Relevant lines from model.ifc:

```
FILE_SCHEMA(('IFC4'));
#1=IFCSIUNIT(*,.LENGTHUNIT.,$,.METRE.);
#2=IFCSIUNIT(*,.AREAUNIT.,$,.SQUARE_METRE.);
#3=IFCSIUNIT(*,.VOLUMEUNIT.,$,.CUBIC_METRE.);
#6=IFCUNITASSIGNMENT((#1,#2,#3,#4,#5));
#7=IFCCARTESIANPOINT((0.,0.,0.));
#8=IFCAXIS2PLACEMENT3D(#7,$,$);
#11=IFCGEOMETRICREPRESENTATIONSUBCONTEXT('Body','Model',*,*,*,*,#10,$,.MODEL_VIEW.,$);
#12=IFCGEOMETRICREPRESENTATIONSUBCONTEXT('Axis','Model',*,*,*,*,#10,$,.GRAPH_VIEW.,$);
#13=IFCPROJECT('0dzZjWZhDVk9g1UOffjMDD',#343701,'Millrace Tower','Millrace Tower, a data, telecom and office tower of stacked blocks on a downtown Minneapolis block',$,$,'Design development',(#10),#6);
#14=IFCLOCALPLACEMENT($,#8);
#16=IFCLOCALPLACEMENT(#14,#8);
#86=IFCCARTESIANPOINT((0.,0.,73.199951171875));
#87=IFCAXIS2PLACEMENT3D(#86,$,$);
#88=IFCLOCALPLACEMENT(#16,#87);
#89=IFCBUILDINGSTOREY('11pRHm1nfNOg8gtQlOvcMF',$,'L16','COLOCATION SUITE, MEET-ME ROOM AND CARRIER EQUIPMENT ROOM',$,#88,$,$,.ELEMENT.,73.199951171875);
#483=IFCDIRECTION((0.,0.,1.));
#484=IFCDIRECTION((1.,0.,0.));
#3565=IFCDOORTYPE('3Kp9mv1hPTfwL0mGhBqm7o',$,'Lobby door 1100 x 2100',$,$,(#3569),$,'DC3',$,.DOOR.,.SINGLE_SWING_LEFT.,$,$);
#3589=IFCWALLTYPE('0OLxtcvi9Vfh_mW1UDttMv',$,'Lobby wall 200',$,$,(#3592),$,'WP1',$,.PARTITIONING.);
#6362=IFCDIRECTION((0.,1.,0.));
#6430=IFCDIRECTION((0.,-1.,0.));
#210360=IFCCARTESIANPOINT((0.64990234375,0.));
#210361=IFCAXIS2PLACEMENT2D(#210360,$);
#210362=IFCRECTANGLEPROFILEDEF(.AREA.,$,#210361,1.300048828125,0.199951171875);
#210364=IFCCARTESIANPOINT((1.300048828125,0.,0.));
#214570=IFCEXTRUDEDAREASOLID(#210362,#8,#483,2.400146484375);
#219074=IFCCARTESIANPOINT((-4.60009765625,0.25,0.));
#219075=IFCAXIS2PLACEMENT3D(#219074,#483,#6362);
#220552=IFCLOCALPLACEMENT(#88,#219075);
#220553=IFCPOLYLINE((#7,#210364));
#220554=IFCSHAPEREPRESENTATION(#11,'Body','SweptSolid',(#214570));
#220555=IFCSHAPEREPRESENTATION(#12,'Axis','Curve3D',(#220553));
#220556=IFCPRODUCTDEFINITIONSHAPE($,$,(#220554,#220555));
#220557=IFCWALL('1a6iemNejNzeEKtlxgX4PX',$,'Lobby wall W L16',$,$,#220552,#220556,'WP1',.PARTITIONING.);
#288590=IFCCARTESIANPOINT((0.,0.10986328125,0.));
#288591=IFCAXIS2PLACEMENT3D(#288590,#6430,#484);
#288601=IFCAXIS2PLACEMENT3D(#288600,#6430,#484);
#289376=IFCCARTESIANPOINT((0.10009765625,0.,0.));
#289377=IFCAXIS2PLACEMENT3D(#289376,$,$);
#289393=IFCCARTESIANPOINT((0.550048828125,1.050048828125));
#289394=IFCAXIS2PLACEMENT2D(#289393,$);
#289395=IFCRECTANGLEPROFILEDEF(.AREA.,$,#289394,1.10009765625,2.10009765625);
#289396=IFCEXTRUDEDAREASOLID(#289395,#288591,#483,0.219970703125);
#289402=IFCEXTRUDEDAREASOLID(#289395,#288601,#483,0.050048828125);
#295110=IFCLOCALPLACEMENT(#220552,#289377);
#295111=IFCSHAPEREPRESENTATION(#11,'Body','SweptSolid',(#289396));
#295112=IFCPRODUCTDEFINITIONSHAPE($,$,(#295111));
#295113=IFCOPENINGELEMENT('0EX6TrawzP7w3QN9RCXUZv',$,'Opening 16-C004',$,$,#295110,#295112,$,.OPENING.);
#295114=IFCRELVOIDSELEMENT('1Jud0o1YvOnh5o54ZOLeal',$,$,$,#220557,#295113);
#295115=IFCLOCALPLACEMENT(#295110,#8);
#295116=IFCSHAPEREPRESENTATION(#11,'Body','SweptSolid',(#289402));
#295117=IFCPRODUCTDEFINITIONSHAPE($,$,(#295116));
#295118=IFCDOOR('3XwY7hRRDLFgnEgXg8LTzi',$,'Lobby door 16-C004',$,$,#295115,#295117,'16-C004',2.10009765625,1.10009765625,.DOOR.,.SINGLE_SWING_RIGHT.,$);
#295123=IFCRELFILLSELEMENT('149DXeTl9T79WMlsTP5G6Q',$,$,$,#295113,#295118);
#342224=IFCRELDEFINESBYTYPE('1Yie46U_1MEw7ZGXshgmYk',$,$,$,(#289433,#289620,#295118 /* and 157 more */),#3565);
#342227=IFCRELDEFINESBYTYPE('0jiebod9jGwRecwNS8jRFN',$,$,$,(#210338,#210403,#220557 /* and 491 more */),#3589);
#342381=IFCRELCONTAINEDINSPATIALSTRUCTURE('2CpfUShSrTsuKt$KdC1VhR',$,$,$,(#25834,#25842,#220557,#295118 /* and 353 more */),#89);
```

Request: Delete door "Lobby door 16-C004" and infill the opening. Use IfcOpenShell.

```python
import ifcopenshell
import ifcopenshell.api.feature
import ifcopenshell.api.root
import ifcopenshell.geom
import ifcopenshell.util.shape

model = ifcopenshell.open("model.ifc")
settings = ifcopenshell.geom.settings()


def volume(element):
    """Net volume in cubic metres, openings subtracted."""
    shape = ifcopenshell.geom.create_shape(settings, element)
    return ifcopenshell.util.shape.get_volume(shape.geometry)


door = model.by_guid("3XwY7hRRDLFgnEgXg8LTzi")
opening = door.FillsVoids[0].RelatingOpeningElement
wall = opening.VoidsElements[0].RelatingBuildingElement
before = volume(wall)

ifcopenshell.api.root.remove_product(model, product=door)
ifcopenshell.api.feature.remove_feature(model, feature=opening)

after = volume(wall)

print(f"wall volume {before:.3f} -> {after:.3f} m3")

model.write("model_rev.ifc")
```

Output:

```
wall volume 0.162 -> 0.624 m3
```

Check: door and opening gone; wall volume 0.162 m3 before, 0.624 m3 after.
